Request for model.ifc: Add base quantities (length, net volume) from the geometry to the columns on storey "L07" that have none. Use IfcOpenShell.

First a look at what the model holds.

```python
import ifcopenshell
import ifcopenshell.util.element
import ifcopenshell.util.unit

model = ifcopenshell.open("model.ifc")
print(model.schema)
for unit_type in ("LENGTHUNIT", "AREAUNIT", "VOLUMEUNIT"):
    print(unit_type, ifcopenshell.util.unit.calculate_unit_scale(model, unit_type))
storey = next(s for s in model.by_type("IfcBuildingStorey") if s.Name == "L07")
columns = [e for e in ifcopenshell.util.element.get_decomposition(storey) if e.is_a("IfcColumn")]
for e in sorted(columns, key=lambda e: e.id()):
    print(e.id(), e.is_a(), e.Name, list(ifcopenshell.util.element.get_psets(e, qtos_only=True)), sep=" | ")
```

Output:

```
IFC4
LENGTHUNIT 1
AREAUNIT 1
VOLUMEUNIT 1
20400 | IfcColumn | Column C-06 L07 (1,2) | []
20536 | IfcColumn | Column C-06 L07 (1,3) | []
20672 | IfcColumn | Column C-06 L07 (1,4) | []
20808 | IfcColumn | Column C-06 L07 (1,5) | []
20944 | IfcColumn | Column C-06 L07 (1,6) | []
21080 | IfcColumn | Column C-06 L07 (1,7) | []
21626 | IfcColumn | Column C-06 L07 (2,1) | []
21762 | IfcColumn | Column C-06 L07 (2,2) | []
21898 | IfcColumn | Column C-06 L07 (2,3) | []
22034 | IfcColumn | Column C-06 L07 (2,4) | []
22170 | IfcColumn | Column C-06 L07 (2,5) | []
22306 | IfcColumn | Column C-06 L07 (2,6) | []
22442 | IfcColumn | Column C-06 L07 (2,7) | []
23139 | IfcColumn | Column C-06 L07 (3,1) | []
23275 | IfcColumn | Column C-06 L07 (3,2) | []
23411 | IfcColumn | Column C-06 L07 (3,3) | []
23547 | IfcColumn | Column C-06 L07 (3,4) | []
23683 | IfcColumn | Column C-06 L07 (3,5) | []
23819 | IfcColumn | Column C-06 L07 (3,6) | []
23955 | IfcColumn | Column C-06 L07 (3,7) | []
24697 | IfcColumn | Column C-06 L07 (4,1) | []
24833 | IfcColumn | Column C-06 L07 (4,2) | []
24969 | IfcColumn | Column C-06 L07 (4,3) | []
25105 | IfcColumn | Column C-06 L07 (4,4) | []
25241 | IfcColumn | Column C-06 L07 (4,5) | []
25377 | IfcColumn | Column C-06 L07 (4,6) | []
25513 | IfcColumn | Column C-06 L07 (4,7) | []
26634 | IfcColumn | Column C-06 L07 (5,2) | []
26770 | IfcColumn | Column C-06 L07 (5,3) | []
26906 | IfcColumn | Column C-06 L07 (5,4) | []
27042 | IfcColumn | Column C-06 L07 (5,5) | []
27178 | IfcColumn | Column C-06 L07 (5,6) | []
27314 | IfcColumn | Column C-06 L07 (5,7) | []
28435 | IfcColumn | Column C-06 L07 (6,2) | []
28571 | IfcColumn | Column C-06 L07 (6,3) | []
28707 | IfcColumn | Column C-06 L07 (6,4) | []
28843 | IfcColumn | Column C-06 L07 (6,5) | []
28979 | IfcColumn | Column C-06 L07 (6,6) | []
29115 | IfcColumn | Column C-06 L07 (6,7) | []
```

```python
import ifcopenshell
import ifcopenshell.api.pset
import ifcopenshell.geom
import ifcopenshell.util.element
import ifcopenshell.util.shape
import ifcopenshell.util.unit

model = ifcopenshell.open("model.ifc")
unit_scale = ifcopenshell.util.unit.calculate_unit_scale(model)
volume_scale = ifcopenshell.util.unit.calculate_unit_scale(model, "VOLUMEUNIT")
settings = ifcopenshell.geom.settings()

storey = next(s for s in model.by_type("IfcBuildingStorey") if s.Name == "L07")
columns = [e for e in ifcopenshell.util.element.get_decomposition(storey) if e.is_a("IfcColumn")]

for e in sorted(columns, key=lambda e: e.id()):
    if ifcopenshell.util.element.get_psets(e, qtos_only=True, should_inherit=False):
        continue
    # Geometry comes back in metres, in the element's own axes.
    shape = ifcopenshell.geom.create_shape(settings, e)
    values = {
        "Length": ifcopenshell.util.shape.get_z(shape.geometry) / unit_scale,
        "NetVolume": ifcopenshell.util.shape.get_volume(shape.geometry) / volume_scale,
    }
    qto = ifcopenshell.api.pset.add_qto(model, product=e, name="Qto_ColumnBaseQuantities")
    ifcopenshell.api.pset.edit_qto(model, qto=qto, properties=values)
    print(e.id(), {k: round(v, 3) for k, v in values.items()})

model.write("model_edited.ifc")
```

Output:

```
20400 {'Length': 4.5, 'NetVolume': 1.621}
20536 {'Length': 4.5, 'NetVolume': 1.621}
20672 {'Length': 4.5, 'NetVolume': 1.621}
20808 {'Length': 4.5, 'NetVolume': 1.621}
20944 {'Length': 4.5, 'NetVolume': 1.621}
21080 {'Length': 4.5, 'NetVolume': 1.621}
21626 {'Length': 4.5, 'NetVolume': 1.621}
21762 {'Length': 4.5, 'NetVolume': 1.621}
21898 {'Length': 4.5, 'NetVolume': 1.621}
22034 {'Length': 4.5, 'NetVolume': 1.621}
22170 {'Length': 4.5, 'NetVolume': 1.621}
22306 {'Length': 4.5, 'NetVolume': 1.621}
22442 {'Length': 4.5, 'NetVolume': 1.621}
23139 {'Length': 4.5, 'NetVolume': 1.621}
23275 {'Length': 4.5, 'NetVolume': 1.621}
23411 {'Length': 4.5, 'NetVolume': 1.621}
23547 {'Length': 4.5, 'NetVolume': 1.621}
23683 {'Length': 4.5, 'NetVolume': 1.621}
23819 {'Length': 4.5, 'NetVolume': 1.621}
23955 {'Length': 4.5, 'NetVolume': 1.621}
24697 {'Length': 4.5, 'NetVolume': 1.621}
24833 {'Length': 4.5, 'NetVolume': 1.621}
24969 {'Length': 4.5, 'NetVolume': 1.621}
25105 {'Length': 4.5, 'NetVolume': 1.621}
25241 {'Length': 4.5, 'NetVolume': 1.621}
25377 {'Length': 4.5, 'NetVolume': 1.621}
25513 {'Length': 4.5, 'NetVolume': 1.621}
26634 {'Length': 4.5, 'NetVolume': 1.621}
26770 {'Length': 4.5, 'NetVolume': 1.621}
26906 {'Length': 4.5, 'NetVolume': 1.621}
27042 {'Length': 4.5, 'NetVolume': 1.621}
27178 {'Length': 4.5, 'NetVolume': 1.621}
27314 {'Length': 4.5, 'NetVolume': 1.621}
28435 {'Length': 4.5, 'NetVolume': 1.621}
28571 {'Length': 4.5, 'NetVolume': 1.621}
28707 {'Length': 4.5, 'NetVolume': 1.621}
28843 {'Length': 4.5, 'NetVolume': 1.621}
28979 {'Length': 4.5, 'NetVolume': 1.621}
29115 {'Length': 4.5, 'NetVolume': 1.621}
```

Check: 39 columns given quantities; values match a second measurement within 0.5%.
